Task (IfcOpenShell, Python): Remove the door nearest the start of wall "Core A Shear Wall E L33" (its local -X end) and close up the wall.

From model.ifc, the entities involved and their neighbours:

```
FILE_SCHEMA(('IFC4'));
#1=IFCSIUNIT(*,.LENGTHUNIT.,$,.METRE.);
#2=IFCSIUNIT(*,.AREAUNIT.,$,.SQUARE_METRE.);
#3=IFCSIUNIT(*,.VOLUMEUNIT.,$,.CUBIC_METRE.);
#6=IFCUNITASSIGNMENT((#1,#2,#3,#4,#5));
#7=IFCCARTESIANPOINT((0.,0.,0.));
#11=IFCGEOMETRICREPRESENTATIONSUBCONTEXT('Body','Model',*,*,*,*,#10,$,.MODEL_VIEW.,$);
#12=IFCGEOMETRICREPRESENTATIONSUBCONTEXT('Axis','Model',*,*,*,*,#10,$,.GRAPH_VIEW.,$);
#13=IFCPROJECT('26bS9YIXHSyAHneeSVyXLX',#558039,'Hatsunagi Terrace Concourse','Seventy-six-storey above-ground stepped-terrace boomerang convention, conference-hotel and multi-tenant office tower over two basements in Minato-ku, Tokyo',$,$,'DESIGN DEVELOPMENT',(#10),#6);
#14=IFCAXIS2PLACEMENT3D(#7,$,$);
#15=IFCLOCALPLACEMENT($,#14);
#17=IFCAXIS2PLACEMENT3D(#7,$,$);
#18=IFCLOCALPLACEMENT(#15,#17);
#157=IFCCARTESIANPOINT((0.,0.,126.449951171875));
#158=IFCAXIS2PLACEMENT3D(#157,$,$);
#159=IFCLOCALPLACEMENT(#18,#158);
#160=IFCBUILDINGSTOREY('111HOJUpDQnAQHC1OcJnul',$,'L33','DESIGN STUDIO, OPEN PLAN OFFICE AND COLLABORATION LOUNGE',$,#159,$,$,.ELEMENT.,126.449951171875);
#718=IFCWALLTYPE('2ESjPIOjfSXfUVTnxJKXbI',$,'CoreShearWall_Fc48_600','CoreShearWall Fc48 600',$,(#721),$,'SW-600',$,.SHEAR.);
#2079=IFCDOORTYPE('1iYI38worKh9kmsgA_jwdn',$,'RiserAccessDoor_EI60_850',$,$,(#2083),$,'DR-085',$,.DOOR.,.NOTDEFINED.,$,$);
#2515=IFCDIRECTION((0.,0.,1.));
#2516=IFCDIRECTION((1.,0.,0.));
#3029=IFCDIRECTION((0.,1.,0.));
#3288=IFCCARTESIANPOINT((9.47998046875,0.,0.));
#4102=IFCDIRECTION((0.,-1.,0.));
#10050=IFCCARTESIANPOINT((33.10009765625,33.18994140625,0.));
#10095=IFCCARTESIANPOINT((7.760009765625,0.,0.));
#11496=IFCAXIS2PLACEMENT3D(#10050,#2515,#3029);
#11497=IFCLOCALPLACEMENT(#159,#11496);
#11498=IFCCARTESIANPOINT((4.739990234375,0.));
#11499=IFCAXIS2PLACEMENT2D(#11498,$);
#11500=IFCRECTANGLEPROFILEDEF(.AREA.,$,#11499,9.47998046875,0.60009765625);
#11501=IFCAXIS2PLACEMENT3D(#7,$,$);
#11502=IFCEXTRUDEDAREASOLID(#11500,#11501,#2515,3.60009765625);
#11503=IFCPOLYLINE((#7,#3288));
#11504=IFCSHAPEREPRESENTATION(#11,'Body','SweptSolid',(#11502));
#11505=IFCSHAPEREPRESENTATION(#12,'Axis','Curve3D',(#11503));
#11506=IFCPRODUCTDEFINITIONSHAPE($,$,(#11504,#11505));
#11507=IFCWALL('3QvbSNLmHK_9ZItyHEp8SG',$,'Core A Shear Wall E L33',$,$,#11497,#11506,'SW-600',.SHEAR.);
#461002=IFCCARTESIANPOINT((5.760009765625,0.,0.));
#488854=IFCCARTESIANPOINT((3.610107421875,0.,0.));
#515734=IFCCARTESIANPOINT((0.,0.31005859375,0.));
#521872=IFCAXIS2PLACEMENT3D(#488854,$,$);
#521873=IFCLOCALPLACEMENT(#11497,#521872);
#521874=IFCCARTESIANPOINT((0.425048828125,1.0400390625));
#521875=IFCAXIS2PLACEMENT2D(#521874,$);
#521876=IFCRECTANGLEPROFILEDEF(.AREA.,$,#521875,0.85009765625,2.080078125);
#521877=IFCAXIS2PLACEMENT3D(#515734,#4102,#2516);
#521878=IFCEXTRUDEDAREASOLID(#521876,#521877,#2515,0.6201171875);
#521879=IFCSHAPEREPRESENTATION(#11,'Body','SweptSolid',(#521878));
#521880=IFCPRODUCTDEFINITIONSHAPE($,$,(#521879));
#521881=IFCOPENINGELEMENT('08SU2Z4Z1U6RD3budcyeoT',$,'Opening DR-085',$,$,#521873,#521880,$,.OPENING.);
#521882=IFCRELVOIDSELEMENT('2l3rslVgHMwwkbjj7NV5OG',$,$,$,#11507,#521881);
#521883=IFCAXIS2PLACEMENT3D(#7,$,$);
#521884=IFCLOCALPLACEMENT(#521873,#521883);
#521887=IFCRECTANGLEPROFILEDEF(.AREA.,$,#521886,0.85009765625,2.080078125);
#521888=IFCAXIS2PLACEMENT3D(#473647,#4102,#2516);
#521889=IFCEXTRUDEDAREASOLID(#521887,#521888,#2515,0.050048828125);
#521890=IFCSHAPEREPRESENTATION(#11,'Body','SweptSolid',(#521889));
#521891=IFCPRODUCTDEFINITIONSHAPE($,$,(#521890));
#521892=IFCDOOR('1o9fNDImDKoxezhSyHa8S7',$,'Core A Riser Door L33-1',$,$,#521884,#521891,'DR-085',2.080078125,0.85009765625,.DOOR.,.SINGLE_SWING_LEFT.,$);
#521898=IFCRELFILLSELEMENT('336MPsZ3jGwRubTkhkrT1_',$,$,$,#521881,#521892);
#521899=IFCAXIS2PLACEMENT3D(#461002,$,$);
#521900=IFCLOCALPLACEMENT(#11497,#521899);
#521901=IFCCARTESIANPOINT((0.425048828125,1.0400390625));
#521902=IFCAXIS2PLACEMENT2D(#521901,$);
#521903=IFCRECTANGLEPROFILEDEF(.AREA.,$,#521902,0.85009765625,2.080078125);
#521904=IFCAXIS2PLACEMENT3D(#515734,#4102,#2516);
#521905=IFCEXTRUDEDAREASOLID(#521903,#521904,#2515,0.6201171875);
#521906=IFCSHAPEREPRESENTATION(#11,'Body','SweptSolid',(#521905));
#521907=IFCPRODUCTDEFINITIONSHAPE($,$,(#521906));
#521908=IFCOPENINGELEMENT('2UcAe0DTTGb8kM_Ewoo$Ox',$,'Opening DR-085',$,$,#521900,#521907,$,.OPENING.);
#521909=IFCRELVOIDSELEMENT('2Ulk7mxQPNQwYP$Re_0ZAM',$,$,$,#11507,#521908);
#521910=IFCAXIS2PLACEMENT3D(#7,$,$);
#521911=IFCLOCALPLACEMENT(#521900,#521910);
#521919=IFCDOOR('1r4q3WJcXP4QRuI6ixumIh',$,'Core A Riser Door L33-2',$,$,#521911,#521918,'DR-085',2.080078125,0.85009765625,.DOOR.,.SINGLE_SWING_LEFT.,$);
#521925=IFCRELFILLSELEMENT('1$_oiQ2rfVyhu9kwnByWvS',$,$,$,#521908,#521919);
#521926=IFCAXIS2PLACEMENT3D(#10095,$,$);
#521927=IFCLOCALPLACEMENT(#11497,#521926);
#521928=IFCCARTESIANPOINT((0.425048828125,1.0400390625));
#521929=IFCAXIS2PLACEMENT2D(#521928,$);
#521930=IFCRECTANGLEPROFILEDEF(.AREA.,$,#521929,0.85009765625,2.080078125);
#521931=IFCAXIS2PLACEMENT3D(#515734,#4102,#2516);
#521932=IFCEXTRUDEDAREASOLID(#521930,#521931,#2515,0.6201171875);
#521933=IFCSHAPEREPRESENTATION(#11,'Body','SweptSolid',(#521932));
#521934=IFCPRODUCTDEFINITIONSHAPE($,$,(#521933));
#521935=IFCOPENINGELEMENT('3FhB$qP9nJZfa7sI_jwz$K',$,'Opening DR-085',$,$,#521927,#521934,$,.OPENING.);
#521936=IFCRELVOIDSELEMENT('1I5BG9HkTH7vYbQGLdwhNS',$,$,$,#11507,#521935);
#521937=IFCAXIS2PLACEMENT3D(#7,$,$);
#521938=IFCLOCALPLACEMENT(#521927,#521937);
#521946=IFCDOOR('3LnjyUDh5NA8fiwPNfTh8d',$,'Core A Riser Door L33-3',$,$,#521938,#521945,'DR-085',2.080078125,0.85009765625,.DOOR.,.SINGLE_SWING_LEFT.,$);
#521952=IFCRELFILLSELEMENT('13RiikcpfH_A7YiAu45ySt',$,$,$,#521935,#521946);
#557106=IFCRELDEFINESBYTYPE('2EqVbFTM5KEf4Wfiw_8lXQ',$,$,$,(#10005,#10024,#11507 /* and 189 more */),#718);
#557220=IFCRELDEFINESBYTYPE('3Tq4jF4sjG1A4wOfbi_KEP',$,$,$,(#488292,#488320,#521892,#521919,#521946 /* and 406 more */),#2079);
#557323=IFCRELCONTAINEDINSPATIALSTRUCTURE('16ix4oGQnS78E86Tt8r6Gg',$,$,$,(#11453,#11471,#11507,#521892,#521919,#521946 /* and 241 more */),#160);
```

```python
import ifcopenshell
import ifcopenshell.api.feature
import ifcopenshell.api.root
import ifcopenshell.geom
import ifcopenshell.util.shape

model = ifcopenshell.open("model.ifc")
settings = ifcopenshell.geom.settings()


def volume(element):
    """Net volume in cubic metres, openings subtracted."""
    shape = ifcopenshell.geom.create_shape(settings, element)
    return ifcopenshell.util.shape.get_volume(shape.geometry)


door = model.by_guid("1o9fNDImDKoxezhSyHa8S7")
opening = door.FillsVoids[0].RelatingOpeningElement
wall = opening.VoidsElements[0].RelatingBuildingElement
before = volume(wall)

ifcopenshell.api.root.remove_product(model, product=door)
ifcopenshell.api.feature.remove_feature(model, feature=opening)

after = volume(wall)

print(f"wall volume {before:.3f} -> {after:.3f} m3")

model.write("model-out.ifc")
```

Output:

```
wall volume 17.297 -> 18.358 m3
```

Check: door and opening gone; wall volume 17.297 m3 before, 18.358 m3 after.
